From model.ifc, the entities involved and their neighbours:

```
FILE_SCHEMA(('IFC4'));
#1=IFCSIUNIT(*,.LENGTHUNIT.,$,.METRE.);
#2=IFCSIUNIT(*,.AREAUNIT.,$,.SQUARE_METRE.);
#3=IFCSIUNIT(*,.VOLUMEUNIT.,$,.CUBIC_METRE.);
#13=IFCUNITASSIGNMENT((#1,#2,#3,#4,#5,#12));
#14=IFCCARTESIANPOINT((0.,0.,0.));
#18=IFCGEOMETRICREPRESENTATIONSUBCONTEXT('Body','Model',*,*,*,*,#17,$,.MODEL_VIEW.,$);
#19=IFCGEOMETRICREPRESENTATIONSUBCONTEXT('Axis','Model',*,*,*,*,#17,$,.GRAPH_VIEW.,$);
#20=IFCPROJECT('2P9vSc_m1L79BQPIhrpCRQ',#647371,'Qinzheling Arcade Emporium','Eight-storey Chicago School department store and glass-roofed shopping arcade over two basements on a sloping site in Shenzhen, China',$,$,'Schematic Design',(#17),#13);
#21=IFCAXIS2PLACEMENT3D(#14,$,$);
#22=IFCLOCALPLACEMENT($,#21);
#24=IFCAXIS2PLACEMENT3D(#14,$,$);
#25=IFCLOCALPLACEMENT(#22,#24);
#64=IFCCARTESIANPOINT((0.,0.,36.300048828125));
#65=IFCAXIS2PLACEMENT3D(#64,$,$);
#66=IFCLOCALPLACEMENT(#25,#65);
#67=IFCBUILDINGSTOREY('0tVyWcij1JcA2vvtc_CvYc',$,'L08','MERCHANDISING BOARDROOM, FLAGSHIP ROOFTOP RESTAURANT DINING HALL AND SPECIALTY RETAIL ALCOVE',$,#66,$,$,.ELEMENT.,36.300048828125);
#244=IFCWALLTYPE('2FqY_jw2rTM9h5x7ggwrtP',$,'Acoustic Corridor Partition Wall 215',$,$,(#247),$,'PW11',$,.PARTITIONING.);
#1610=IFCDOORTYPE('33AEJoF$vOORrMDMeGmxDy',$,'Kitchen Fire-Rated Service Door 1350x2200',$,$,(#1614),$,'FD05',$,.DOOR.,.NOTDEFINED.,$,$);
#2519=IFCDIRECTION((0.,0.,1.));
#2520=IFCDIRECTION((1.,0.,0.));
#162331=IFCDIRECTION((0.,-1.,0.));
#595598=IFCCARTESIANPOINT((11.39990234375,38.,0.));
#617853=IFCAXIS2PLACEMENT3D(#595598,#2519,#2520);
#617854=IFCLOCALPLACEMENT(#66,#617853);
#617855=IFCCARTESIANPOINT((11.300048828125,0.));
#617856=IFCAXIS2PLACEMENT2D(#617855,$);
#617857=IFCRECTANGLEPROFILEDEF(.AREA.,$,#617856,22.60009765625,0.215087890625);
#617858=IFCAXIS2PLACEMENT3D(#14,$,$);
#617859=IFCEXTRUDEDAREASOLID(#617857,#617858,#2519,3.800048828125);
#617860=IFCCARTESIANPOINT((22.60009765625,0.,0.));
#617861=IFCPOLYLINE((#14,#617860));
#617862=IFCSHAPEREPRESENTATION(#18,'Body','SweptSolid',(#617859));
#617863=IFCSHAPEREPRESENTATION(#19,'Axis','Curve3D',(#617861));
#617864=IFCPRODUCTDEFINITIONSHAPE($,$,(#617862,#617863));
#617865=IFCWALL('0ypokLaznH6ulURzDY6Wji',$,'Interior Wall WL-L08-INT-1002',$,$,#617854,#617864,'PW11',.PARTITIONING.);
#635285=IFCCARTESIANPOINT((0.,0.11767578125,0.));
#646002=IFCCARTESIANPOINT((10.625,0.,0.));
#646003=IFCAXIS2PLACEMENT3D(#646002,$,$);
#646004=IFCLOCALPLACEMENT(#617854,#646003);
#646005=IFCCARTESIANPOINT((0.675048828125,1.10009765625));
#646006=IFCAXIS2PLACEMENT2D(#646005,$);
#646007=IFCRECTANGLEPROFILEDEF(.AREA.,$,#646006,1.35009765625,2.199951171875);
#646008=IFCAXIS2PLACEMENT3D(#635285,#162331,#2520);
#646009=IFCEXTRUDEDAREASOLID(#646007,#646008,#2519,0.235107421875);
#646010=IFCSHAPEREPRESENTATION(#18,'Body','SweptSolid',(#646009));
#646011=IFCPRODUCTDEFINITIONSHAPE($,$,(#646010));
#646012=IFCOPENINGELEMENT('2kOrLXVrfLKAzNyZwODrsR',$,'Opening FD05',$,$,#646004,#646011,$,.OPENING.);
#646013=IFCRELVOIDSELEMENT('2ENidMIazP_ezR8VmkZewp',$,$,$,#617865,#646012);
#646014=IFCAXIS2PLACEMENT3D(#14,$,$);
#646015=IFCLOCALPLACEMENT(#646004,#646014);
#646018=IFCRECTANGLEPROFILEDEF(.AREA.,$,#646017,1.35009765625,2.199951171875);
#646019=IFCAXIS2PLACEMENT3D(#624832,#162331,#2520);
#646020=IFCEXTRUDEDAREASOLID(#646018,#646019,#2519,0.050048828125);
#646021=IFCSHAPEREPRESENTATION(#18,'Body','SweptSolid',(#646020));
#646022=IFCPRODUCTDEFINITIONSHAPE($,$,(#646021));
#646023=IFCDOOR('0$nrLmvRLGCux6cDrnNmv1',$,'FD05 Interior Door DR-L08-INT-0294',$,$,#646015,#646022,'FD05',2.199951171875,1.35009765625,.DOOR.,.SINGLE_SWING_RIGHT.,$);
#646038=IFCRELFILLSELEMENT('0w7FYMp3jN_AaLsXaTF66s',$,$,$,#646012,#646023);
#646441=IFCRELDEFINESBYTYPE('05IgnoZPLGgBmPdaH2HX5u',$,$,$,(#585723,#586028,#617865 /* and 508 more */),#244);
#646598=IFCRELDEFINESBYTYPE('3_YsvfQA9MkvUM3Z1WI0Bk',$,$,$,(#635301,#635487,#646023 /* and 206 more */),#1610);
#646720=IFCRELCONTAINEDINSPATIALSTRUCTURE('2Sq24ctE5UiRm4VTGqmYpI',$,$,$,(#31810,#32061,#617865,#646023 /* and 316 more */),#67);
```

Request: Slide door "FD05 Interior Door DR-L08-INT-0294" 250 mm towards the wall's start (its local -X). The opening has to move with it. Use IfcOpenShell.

```python
import ifcopenshell
import ifcopenshell.api.geometry
import ifcopenshell.util.placement

model = ifcopenshell.open("model.ifc")

door = model.by_guid("0$nrLmvRLGCux6cDrnNmv1")
opening = door.FillsVoids[0].RelatingOpeningElement
wall = opening.VoidsElements[0].RelatingBuildingElement

wall_matrix = ifcopenshell.util.placement.get_local_placement(wall.ObjectPlacement)
shift = wall_matrix[:3, 0] * -0.25
before = ifcopenshell.util.placement.get_local_placement(door.ObjectPlacement)[:3, 3].copy()

# The door is placed relative to its opening, so it follows when the opening moves.
matrix = ifcopenshell.util.placement.get_local_placement(opening.ObjectPlacement)
matrix[:3, 3] += shift
ifcopenshell.api.geometry.edit_object_placement(
    model, product=opening, matrix=matrix, is_si=False, should_transform_children=True
)

after = ifcopenshell.util.placement.get_local_placement(door.ObjectPlacement)[:3, 3]
print("door moved by", (after - before).round(3) + 0.0)

model.write("model_edited.ifc")
```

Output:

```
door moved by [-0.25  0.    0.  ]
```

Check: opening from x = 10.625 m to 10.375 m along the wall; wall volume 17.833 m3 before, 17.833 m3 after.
